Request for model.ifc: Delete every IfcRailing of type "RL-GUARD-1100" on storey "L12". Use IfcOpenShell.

First a look at what the model holds.

```python
import ifcopenshell
import ifcopenshell.util.element

model = ifcopenshell.open("model.ifc")
print(model.schema)
storey = next(s for s in model.by_type("IfcBuildingStorey") if s.Name == "L12")
railings = [e for e in ifcopenshell.util.element.get_decomposition(storey) if e.is_a("IfcRailing")]
seen = {}
for e in railings:
    element_type = ifcopenshell.util.element.get_type(e)
    name = element_type.Name if element_type not in (None, e) else None
    seen[name] = seen.get(name, 0) + 1
for name, count in sorted(seen.items(), key=str):
    print(count, "x", name)
```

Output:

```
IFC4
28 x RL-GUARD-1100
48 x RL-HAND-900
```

```python
import ifcopenshell
import ifcopenshell.api.root
import ifcopenshell.util.element

model = ifcopenshell.open("model.ifc")

storey = next(s for s in model.by_type("IfcBuildingStorey") if s.Name == "L12")
railings = [e for e in ifcopenshell.util.element.get_decomposition(storey) if e.is_a("IfcRailing")]
targets = [e for e in railings if (t := ifcopenshell.util.element.get_type(e)) not in (None, e) and t.Name == "RL-GUARD-1100"]

for e in targets:
    ifcopenshell.api.root.remove_product(model, product=e)
print(len(targets), "removed")

model.write("model_edited.ifc")
```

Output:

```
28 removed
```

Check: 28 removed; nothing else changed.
